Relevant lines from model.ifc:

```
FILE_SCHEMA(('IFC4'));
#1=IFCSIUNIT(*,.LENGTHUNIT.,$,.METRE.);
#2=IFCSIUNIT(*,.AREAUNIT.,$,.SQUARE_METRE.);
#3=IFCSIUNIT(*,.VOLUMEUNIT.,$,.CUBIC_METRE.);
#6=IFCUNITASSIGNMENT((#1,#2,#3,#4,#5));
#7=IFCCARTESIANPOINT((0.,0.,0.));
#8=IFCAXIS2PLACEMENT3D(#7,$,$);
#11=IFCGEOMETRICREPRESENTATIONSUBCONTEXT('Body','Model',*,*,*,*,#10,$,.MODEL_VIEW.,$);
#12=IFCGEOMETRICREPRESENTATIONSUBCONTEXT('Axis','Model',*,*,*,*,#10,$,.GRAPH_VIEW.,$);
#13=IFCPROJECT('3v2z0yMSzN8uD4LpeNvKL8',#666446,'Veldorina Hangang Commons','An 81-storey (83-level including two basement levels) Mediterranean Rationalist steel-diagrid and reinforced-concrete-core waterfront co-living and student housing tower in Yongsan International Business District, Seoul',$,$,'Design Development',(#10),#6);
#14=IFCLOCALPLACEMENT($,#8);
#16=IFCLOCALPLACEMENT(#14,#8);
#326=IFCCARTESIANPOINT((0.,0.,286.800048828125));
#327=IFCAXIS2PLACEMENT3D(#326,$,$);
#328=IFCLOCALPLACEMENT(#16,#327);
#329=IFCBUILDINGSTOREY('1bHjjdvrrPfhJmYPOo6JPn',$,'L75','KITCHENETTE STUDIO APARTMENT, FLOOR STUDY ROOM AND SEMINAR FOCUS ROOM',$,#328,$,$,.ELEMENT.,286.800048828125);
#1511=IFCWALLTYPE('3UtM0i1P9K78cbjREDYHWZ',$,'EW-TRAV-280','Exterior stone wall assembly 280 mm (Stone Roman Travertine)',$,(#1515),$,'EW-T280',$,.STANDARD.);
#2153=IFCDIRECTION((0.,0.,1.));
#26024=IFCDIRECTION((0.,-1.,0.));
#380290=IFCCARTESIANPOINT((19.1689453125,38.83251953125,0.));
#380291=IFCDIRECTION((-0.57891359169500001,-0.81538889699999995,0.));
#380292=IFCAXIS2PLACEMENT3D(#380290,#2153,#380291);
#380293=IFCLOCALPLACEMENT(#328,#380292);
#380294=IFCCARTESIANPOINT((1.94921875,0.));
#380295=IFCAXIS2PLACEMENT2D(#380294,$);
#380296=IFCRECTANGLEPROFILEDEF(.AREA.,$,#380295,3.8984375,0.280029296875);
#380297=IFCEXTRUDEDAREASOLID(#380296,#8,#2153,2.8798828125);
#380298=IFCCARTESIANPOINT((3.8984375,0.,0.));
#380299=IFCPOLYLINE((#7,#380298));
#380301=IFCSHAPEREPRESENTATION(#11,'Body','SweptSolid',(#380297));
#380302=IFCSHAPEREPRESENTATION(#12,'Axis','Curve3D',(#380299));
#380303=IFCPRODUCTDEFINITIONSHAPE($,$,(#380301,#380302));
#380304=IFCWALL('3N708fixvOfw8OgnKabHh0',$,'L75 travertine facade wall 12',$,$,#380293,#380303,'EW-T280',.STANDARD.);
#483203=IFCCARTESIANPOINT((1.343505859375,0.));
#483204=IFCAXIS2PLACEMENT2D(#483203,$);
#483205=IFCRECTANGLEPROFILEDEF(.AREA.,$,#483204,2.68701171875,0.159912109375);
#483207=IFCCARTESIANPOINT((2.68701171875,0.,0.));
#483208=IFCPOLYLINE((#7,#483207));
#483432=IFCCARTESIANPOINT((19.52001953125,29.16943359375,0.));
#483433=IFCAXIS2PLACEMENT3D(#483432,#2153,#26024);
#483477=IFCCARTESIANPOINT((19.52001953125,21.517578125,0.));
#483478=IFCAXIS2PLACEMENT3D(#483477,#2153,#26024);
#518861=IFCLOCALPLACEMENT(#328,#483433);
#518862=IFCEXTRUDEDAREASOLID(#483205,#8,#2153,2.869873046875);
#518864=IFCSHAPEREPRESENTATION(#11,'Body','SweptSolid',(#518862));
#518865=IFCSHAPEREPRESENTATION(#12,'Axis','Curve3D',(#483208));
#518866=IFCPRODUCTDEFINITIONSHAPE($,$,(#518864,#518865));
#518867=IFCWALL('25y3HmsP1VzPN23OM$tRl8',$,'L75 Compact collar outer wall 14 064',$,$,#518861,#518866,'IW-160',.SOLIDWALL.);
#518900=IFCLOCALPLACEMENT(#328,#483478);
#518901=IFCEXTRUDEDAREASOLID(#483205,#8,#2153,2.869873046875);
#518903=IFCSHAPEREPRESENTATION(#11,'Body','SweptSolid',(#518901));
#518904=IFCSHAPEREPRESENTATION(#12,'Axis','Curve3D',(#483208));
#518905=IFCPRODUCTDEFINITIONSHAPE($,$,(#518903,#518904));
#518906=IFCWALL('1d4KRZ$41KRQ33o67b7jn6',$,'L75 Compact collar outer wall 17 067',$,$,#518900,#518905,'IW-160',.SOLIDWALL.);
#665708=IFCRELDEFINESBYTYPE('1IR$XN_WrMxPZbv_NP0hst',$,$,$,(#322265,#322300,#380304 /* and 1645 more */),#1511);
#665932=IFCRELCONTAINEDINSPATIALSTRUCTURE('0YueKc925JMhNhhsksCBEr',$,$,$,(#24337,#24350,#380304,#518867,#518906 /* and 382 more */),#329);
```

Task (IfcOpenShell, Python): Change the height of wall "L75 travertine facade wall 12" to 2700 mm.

```python
import ifcopenshell
import ifcopenshell.geom
import ifcopenshell.util.representation
import ifcopenshell.util.shape

model = ifcopenshell.open("model.ifc")
settings = ifcopenshell.geom.settings()


def volume(element):
    """Net volume in cubic metres, openings subtracted."""
    shape = ifcopenshell.geom.create_shape(settings, element)
    return ifcopenshell.util.shape.get_volume(shape.geometry)


wall = model.by_id(380304)
before = volume(wall)

body = ifcopenshell.util.representation.get_representation(wall, "Model", "Body")
solid = body.Items[0]
old_height = solid.Depth
solid.Depth = 2.7
after = volume(wall)

print(f"height {old_height:g} -> {solid.Depth:g}, volume {before:.3f} -> {after:.3f} m3")

model.write("model-out.ifc")
```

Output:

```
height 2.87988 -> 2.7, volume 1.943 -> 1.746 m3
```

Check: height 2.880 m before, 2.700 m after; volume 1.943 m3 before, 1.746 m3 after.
